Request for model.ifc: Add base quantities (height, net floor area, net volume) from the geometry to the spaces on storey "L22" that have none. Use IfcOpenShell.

First a look at what the model holds.

```python
import ifcopenshell
import ifcopenshell.util.element
import ifcopenshell.util.unit

model = ifcopenshell.open("model.ifc")
print(model.schema)
for unit_type in ("LENGTHUNIT", "AREAUNIT", "VOLUMEUNIT"):
    print(unit_type, ifcopenshell.util.unit.calculate_unit_scale(model, unit_type))
storey = next(s for s in model.by_type("IfcBuildingStorey") if s.Name == "L22")
spaces = [e for e in ifcopenshell.util.element.get_decomposition(storey) if e.is_a("IfcSpace")]
for e in sorted(spaces, key=lambda e: e.id()):
    print(e.id(), e.is_a(), e.Name, list(ifcopenshell.util.element.get_psets(e, qtos_only=True)), sep=" | ")
```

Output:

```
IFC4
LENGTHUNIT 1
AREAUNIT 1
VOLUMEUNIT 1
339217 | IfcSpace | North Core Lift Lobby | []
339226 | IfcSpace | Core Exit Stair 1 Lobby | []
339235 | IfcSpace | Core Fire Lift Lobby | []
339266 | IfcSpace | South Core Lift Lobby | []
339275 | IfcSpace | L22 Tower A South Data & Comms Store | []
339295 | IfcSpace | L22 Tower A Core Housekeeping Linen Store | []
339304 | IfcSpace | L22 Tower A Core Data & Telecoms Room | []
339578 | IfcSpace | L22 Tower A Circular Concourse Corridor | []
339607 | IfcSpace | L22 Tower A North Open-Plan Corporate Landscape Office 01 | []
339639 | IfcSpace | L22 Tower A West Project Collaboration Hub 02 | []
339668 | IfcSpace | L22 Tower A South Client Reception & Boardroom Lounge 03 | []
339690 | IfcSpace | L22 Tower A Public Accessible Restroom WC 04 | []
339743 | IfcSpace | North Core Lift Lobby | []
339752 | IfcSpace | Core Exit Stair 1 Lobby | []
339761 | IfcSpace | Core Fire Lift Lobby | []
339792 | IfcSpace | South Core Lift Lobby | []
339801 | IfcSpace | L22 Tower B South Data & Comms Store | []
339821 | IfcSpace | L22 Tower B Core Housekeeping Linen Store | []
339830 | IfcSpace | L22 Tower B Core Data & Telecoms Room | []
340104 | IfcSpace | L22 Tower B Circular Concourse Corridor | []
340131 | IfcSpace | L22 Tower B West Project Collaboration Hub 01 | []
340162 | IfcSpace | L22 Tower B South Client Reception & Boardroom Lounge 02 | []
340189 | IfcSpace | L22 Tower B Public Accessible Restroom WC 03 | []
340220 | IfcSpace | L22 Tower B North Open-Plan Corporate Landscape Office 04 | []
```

```python
import ifcopenshell
import ifcopenshell.api.pset
import ifcopenshell.geom
import ifcopenshell.util.element
import ifcopenshell.util.shape
import ifcopenshell.util.unit

model = ifcopenshell.open("model.ifc")
unit_scale = ifcopenshell.util.unit.calculate_unit_scale(model)
area_scale = ifcopenshell.util.unit.calculate_unit_scale(model, "AREAUNIT")
volume_scale = ifcopenshell.util.unit.calculate_unit_scale(model, "VOLUMEUNIT")
settings = ifcopenshell.geom.settings()

storey = next(s for s in model.by_type("IfcBuildingStorey") if s.Name == "L22")
spaces = [e for e in ifcopenshell.util.element.get_decomposition(storey) if e.is_a("IfcSpace")]

for e in sorted(spaces, key=lambda e: e.id()):
    if ifcopenshell.util.element.get_psets(e, qtos_only=True, should_inherit=False):
        continue
    # Geometry comes back in metres, in the element's own axes.
    shape = ifcopenshell.geom.create_shape(settings, e)
    values = {
        "Height": ifcopenshell.util.shape.get_z(shape.geometry) / unit_scale,
        "NetFloorArea": ifcopenshell.util.shape.get_footprint_area(shape.geometry) / area_scale,
        "NetVolume": ifcopenshell.util.shape.get_volume(shape.geometry) / volume_scale,
    }
    qto = ifcopenshell.api.pset.add_qto(model, product=e, name="Qto_SpaceBaseQuantities")
    ifcopenshell.api.pset.edit_qto(model, qto=qto, properties=values)
    print(e.id(), {k: round(v, 3) for k, v in values.items()})

model.write("model-out.ifc")
```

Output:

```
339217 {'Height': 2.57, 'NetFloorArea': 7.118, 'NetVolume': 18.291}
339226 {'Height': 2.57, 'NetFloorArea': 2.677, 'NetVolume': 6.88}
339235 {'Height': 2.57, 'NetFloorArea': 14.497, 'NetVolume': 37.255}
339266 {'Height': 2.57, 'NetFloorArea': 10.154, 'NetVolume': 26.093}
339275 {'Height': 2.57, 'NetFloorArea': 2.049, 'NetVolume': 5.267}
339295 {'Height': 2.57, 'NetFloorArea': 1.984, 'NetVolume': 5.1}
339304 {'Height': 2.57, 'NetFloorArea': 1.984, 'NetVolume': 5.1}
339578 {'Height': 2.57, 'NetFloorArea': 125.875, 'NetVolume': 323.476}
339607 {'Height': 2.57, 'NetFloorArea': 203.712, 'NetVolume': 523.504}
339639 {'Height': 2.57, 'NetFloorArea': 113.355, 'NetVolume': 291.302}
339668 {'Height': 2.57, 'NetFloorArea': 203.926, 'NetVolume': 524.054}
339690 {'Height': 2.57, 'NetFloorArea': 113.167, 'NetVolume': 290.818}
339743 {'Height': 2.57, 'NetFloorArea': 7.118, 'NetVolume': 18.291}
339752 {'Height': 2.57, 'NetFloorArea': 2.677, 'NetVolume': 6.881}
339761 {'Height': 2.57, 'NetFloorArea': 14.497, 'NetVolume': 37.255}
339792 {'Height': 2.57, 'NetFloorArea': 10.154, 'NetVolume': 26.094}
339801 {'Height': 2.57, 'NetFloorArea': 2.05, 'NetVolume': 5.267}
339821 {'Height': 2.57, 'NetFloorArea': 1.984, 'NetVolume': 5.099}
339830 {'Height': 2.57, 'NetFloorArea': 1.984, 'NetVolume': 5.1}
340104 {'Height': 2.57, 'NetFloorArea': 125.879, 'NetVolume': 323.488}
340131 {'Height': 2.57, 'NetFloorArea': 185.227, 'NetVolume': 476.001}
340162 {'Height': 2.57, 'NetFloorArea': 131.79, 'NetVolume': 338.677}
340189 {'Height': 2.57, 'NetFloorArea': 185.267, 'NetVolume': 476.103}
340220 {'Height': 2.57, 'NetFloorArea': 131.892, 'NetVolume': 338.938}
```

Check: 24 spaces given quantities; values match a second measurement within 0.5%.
